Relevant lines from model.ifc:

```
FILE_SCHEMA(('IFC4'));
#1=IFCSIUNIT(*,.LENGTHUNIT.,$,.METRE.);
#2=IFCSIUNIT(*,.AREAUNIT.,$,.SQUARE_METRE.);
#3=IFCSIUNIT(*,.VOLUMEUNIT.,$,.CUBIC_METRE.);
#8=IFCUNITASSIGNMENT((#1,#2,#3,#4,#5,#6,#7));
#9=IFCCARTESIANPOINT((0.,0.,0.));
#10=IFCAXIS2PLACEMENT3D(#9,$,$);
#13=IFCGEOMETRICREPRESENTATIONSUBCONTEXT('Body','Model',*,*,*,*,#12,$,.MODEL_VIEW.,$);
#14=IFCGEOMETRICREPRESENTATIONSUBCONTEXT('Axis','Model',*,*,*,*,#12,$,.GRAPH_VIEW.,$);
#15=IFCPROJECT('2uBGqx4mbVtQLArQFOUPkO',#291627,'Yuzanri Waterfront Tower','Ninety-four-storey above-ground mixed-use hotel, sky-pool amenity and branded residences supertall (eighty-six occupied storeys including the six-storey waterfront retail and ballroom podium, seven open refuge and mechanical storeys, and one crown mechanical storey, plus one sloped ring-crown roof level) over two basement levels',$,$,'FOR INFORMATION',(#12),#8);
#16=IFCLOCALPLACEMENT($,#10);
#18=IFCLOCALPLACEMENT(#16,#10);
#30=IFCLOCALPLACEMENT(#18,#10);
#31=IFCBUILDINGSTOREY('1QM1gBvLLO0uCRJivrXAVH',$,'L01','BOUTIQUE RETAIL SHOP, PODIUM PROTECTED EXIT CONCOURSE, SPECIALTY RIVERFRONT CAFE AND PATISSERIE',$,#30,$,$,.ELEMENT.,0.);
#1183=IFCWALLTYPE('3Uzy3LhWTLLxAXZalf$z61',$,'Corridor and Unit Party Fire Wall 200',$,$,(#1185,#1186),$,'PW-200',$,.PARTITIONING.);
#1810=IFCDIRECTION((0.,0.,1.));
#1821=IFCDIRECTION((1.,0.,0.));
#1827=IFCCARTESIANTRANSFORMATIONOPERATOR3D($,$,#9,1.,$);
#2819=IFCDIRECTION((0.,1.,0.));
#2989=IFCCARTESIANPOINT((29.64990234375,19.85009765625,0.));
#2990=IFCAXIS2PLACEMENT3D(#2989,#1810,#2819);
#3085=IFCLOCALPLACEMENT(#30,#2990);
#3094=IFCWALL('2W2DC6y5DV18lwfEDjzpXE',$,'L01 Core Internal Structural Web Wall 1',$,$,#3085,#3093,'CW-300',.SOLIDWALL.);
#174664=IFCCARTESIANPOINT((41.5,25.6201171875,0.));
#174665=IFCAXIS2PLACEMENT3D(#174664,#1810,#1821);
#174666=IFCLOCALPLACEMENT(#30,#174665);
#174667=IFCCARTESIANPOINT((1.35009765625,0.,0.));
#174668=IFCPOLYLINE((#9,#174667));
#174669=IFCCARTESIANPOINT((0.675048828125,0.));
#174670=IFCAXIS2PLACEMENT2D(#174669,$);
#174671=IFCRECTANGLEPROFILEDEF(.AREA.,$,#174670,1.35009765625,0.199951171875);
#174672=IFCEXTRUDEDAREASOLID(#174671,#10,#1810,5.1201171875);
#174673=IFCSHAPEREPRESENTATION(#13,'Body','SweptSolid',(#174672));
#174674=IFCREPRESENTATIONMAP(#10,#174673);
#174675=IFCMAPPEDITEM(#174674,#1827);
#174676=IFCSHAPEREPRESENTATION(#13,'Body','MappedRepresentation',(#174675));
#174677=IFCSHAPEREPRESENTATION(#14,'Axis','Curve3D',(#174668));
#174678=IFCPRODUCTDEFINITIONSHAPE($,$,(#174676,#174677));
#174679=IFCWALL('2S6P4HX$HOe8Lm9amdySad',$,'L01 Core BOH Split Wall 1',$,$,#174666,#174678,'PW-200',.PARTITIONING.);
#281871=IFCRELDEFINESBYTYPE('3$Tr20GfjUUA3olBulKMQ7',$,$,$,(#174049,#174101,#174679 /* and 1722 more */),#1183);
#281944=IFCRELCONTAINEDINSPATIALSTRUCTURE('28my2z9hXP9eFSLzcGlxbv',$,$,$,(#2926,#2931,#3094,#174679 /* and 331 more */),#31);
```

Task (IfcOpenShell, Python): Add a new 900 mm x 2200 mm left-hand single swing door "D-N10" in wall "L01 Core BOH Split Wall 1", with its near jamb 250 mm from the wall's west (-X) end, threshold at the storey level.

```python
import numpy as np
import ifcopenshell
import ifcopenshell.api.feature
import ifcopenshell.api.geometry
import ifcopenshell.api.root
import ifcopenshell.api.spatial
import ifcopenshell.geom
import ifcopenshell.util.element
import ifcopenshell.util.placement
import ifcopenshell.util.representation
import ifcopenshell.util.shape
import ifcopenshell.util.unit

model = ifcopenshell.open("model.ifc")
unit_scale = ifcopenshell.util.unit.calculate_unit_scale(model)
settings = ifcopenshell.geom.settings()


def volume(element):
    """Net volume in cubic metres, openings subtracted."""
    shape = ifcopenshell.geom.create_shape(settings, element)
    return ifcopenshell.util.shape.get_volume(shape.geometry)


wall = model.by_guid("2S6P4HX$HOe8Lm9amdySad")
storey = ifcopenshell.util.element.get_container(wall, ifc_class="IfcBuildingStorey")
context = ifcopenshell.util.representation.get_context(model, "Model", "Body", "MODEL_VIEW")
before = volume(wall)

width, height, from_end, sill = 0.9, 2.2, 0.25, 0.0  # metres

# The wall runs along its own X axis, and the end named is its -X end.
wall_shape = ifcopenshell.geom.create_shape(settings, wall)
x, y, z = ifcopenshell.util.shape.get_vertices(wall_shape.geometry).T
start = x.min() + from_end
face, thickness = float(y.min()), float(y.max() - y.min())
wall_matrix = ifcopenshell.util.placement.get_local_placement(wall.ObjectPlacement)
level = ifcopenshell.util.placement.get_local_placement(storey.ObjectPlacement)[2, 3]


def in_wall(x, y):
    """Placement at x, y metres in the wall's axes, at sill height."""
    matrix = wall_matrix.copy()
    matrix[:, 3] = wall_matrix @ np.array([x / unit_scale, y / unit_scale, 0.0, 1.0])
    matrix[2, 3] = level + sill / unit_scale
    return matrix


# Opening: a box that overshoots both wall faces by 50 mm.
opening = ifcopenshell.api.root.create_entity(model, ifc_class="IfcOpeningElement", predefined_type="OPENING")
box = ifcopenshell.api.geometry.add_wall_representation(
    model, context=context, length=width, height=height, thickness=thickness + 0.1
)
ifcopenshell.api.geometry.assign_representation(model, product=opening, representation=box)
ifcopenshell.api.geometry.edit_object_placement(model, product=opening, matrix=in_wall(start, face - 0.05), is_si=False)
ifcopenshell.api.feature.add_feature(model, feature=opening, element=wall)

door = ifcopenshell.api.root.create_entity(model, ifc_class="IfcDoor", name="D-N10", predefined_type="DOOR")
door.OverallWidth, door.OverallHeight = width / unit_scale, height / unit_scale
door.OperationType = "SINGLE_SWING_LEFT"
body = ifcopenshell.api.geometry.add_door_representation(
    model,
    context=context,
    overall_width=door.OverallWidth,
    overall_height=door.OverallHeight,
    operation_type="SINGLE_SWING_LEFT",
    lining_properties={"LiningDepth": thickness / unit_scale, "ThresholdDepth": thickness / unit_scale},
)
ifcopenshell.api.geometry.assign_representation(model, product=door, representation=body)
ifcopenshell.api.spatial.assign_container(model, products=[door], relating_structure=storey)
ifcopenshell.api.feature.add_filling(model, opening=opening, element=door)

# The lining spans the wall, so the door starts at the wall face.
ifcopenshell.api.geometry.edit_object_placement(model, product=door, matrix=in_wall(start, face), is_si=False)

after = volume(wall)

print(f"wall volume {before:.3f} -> {after:.3f} m3")

model.write("model_edited.ifc")
```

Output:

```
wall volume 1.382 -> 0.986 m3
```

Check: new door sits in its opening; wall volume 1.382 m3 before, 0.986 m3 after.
